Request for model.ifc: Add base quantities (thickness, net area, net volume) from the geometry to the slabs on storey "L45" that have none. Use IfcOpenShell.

First a look at what the model holds.

```python
import ifcopenshell
import ifcopenshell.util.element
import ifcopenshell.util.unit

model = ifcopenshell.open("model.ifc")
print(model.schema)
for unit_type in ("LENGTHUNIT", "AREAUNIT", "VOLUMEUNIT"):
    print(unit_type, ifcopenshell.util.unit.calculate_unit_scale(model, unit_type))
storey = next(s for s in model.by_type("IfcBuildingStorey") if s.Name == "L45")
slabs = [e for e in ifcopenshell.util.element.get_decomposition(storey) if e.is_a("IfcSlab")]
for e in sorted(slabs, key=lambda e: e.id()):
    print(e.id(), e.is_a(), e.Name, list(ifcopenshell.util.element.get_psets(e, qtos_only=True)), sep=" | ")
```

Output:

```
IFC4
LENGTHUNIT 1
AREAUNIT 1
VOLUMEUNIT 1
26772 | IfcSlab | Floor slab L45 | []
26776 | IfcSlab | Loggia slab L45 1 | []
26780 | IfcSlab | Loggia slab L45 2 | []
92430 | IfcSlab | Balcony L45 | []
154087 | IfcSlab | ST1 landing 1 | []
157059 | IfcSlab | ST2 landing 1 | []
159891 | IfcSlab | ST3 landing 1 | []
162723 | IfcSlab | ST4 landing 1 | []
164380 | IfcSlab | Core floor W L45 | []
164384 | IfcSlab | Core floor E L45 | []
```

```python
import ifcopenshell
import ifcopenshell.api.pset
import ifcopenshell.geom
import ifcopenshell.util.element
import ifcopenshell.util.shape
import ifcopenshell.util.unit

model = ifcopenshell.open("model.ifc")
unit_scale = ifcopenshell.util.unit.calculate_unit_scale(model)
area_scale = ifcopenshell.util.unit.calculate_unit_scale(model, "AREAUNIT")
volume_scale = ifcopenshell.util.unit.calculate_unit_scale(model, "VOLUMEUNIT")
settings = ifcopenshell.geom.settings()

storey = next(s for s in model.by_type("IfcBuildingStorey") if s.Name == "L45")
slabs = [e for e in ifcopenshell.util.element.get_decomposition(storey) if e.is_a("IfcSlab")]

for e in sorted(slabs, key=lambda e: e.id()):
    if ifcopenshell.util.element.get_psets(e, qtos_only=True, should_inherit=False):
        continue
    # Geometry comes back in metres, in the element's own axes.
    shape = ifcopenshell.geom.create_shape(settings, e)
    values = {
        "Width": ifcopenshell.util.shape.get_z(shape.geometry) / unit_scale,
        "NetArea": ifcopenshell.util.shape.get_footprint_area(shape.geometry) / area_scale,
        "NetVolume": ifcopenshell.util.shape.get_volume(shape.geometry) / volume_scale,
    }
    qto = ifcopenshell.api.pset.add_qto(model, product=e, name="Qto_SlabBaseQuantities")
    ifcopenshell.api.pset.edit_qto(model, qto=qto, properties=values)
    print(e.id(), {k: round(v, 3) for k, v in values.items()})

model.write("model_v2.ifc")
```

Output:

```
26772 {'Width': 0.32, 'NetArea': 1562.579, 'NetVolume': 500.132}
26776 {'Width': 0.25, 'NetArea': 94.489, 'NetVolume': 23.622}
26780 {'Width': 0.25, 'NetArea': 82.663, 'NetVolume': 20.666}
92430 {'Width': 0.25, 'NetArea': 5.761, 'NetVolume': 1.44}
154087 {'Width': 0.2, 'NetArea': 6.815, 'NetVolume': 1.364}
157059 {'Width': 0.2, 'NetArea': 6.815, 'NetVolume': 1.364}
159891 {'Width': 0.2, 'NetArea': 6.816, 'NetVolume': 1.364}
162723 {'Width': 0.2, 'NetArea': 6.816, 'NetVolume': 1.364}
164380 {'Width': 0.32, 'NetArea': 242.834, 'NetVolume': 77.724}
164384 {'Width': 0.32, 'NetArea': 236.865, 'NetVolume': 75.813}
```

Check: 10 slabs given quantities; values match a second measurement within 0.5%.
